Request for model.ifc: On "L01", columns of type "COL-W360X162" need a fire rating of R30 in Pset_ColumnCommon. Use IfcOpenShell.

First a look at what the model holds.

```python
import ifcopenshell
import ifcopenshell.util.element

model = ifcopenshell.open("model.ifc")
print(model.schema)
storey = next(s for s in model.by_type("IfcBuildingStorey") if s.Name == "L01")
columns = [e for e in ifcopenshell.util.element.get_decomposition(storey) if e.is_a("IfcColumn")]
seen = {}
for e in columns:
    element_type = ifcopenshell.util.element.get_type(e)
    key = (element_type.Name if element_type != e and element_type else None, ifcopenshell.util.element.get_pset(e, "Pset_ColumnCommon", "FireRating"))
    seen[key] = seen.get(key, 0) + 1
for (name, value), count in sorted(seen.items(), key=str):
    print(count, "x", name, "|", value)
```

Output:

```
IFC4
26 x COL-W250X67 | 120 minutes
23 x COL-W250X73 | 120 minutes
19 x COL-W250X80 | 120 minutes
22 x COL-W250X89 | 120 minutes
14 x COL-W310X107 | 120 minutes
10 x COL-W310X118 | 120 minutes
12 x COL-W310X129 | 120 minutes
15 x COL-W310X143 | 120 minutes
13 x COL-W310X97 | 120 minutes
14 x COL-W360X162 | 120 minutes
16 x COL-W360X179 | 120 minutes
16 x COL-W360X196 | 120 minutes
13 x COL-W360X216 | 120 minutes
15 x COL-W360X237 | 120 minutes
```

```python
import ifcopenshell
import ifcopenshell.api.pset
import ifcopenshell.util.element

model = ifcopenshell.open("model.ifc")

storey = next(s for s in model.by_type("IfcBuildingStorey") if s.Name == "L01")
columns = [e for e in ifcopenshell.util.element.get_decomposition(storey) if e.is_a("IfcColumn")]

count = 0
for e in columns:
    element_type = ifcopenshell.util.element.get_type(e)
    if element_type in (None, e) or element_type.Name != "COL-W360X162":
        continue
    # add_pset returns the element's existing set when there is one.
    pset = ifcopenshell.api.pset.add_pset(model, product=e, name="Pset_ColumnCommon")
    ifcopenshell.api.pset.edit_pset(model, pset=pset, properties={"FireRating": "R30"})
    count += 1

print(count, "columns updated")

model.write("model_v2.ifc")
```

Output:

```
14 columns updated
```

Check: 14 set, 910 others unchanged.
